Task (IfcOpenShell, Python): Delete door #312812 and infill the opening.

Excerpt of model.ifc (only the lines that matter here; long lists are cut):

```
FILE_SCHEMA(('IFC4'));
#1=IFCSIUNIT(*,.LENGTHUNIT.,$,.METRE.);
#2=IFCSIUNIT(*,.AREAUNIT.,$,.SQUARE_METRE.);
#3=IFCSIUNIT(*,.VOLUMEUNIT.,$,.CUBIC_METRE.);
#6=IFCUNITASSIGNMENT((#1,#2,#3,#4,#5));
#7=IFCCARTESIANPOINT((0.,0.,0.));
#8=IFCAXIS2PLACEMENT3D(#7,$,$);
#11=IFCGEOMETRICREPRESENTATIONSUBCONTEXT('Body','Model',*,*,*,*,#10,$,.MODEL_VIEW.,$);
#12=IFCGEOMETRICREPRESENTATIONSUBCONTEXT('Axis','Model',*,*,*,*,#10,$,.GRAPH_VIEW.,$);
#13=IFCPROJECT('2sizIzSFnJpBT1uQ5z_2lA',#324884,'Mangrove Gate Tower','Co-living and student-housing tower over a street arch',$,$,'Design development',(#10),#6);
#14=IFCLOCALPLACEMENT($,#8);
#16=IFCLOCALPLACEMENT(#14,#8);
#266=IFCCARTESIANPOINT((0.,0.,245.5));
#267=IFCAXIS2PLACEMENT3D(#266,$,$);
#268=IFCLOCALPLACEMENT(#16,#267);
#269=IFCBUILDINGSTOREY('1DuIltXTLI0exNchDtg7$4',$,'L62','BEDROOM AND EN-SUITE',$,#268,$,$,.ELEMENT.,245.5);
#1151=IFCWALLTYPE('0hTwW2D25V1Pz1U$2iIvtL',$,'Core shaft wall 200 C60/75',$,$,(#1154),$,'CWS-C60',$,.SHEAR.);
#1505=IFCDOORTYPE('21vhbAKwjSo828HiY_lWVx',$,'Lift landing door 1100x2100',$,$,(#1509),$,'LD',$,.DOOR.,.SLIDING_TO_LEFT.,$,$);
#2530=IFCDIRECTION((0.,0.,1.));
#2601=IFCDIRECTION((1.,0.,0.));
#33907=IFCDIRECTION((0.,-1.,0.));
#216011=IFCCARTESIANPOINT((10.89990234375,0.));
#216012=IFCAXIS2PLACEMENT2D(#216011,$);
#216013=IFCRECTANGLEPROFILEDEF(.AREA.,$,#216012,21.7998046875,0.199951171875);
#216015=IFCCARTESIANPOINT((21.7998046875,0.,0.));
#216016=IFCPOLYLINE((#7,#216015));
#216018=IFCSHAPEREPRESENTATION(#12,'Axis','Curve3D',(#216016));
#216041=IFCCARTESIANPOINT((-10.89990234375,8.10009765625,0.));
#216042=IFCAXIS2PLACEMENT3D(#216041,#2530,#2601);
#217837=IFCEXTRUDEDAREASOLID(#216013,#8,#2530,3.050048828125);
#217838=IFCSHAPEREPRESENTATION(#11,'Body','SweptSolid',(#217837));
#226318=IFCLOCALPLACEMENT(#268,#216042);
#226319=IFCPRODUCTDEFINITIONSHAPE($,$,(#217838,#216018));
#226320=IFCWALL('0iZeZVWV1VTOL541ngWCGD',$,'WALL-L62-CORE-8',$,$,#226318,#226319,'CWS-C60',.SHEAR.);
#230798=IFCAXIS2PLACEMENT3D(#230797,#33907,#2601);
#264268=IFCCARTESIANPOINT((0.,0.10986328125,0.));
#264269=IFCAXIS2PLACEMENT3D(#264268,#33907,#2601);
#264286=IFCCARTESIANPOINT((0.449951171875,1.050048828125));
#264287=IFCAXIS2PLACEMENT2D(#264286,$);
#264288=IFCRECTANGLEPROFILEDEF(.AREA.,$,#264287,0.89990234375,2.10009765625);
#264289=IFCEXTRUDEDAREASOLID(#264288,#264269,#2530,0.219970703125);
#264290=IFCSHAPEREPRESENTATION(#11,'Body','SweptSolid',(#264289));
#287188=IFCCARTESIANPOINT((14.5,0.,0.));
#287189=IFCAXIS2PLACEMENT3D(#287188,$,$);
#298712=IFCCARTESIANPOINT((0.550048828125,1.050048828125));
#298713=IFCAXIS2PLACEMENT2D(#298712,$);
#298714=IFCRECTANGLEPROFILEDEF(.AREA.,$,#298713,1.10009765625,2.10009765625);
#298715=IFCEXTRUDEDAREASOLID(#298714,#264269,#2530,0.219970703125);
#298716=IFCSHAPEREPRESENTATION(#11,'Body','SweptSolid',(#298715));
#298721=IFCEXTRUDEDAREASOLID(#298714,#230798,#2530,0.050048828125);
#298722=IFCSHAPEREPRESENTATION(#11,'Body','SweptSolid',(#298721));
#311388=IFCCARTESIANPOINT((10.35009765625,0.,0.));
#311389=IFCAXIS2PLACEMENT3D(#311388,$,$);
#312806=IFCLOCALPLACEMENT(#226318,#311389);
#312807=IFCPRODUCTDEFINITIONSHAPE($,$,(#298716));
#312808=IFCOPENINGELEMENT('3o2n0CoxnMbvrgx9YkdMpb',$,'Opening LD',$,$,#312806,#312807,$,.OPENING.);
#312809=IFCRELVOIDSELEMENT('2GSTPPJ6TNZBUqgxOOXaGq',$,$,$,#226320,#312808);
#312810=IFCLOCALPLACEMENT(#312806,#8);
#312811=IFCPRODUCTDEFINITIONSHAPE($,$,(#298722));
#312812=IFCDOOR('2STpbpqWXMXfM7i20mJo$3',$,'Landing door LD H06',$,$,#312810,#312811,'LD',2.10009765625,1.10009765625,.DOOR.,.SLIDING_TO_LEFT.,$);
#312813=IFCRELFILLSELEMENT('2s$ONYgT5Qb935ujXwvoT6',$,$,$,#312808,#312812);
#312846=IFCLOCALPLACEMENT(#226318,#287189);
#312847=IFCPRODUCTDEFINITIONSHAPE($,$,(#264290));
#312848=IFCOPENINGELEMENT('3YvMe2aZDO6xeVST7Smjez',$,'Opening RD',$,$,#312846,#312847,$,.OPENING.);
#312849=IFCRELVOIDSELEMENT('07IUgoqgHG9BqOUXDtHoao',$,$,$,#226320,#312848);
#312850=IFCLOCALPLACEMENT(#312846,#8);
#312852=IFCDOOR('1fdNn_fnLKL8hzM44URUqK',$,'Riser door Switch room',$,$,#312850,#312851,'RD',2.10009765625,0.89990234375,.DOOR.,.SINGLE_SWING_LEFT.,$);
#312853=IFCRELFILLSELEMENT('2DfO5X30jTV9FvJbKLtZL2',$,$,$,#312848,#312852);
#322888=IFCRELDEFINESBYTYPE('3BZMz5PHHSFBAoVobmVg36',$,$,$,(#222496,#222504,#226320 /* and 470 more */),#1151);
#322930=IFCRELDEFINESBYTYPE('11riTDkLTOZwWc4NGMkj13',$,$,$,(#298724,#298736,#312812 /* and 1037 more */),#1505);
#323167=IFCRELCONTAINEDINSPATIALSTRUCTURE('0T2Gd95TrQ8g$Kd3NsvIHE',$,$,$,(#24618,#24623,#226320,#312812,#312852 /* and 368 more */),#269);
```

```python
import ifcopenshell
import ifcopenshell.api.feature
import ifcopenshell.api.root
import ifcopenshell.geom
import ifcopenshell.util.shape

model = ifcopenshell.open("model.ifc")
settings = ifcopenshell.geom.settings()


def volume(element):
    """Net volume in cubic metres, openings subtracted."""
    shape = ifcopenshell.geom.create_shape(settings, element)
    return ifcopenshell.util.shape.get_volume(shape.geometry)


door = model.by_id(312812)
opening = door.FillsVoids[0].RelatingOpeningElement
wall = opening.VoidsElements[0].RelatingBuildingElement
before = volume(wall)

ifcopenshell.api.root.remove_product(model, product=door)
ifcopenshell.api.feature.remove_feature(model, feature=opening)

after = volume(wall)

print(f"wall volume {before:.3f} -> {after:.3f} m3")

model.write("model_rev.ifc")
```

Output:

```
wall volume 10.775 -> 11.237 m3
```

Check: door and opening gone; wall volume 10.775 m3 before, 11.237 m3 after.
